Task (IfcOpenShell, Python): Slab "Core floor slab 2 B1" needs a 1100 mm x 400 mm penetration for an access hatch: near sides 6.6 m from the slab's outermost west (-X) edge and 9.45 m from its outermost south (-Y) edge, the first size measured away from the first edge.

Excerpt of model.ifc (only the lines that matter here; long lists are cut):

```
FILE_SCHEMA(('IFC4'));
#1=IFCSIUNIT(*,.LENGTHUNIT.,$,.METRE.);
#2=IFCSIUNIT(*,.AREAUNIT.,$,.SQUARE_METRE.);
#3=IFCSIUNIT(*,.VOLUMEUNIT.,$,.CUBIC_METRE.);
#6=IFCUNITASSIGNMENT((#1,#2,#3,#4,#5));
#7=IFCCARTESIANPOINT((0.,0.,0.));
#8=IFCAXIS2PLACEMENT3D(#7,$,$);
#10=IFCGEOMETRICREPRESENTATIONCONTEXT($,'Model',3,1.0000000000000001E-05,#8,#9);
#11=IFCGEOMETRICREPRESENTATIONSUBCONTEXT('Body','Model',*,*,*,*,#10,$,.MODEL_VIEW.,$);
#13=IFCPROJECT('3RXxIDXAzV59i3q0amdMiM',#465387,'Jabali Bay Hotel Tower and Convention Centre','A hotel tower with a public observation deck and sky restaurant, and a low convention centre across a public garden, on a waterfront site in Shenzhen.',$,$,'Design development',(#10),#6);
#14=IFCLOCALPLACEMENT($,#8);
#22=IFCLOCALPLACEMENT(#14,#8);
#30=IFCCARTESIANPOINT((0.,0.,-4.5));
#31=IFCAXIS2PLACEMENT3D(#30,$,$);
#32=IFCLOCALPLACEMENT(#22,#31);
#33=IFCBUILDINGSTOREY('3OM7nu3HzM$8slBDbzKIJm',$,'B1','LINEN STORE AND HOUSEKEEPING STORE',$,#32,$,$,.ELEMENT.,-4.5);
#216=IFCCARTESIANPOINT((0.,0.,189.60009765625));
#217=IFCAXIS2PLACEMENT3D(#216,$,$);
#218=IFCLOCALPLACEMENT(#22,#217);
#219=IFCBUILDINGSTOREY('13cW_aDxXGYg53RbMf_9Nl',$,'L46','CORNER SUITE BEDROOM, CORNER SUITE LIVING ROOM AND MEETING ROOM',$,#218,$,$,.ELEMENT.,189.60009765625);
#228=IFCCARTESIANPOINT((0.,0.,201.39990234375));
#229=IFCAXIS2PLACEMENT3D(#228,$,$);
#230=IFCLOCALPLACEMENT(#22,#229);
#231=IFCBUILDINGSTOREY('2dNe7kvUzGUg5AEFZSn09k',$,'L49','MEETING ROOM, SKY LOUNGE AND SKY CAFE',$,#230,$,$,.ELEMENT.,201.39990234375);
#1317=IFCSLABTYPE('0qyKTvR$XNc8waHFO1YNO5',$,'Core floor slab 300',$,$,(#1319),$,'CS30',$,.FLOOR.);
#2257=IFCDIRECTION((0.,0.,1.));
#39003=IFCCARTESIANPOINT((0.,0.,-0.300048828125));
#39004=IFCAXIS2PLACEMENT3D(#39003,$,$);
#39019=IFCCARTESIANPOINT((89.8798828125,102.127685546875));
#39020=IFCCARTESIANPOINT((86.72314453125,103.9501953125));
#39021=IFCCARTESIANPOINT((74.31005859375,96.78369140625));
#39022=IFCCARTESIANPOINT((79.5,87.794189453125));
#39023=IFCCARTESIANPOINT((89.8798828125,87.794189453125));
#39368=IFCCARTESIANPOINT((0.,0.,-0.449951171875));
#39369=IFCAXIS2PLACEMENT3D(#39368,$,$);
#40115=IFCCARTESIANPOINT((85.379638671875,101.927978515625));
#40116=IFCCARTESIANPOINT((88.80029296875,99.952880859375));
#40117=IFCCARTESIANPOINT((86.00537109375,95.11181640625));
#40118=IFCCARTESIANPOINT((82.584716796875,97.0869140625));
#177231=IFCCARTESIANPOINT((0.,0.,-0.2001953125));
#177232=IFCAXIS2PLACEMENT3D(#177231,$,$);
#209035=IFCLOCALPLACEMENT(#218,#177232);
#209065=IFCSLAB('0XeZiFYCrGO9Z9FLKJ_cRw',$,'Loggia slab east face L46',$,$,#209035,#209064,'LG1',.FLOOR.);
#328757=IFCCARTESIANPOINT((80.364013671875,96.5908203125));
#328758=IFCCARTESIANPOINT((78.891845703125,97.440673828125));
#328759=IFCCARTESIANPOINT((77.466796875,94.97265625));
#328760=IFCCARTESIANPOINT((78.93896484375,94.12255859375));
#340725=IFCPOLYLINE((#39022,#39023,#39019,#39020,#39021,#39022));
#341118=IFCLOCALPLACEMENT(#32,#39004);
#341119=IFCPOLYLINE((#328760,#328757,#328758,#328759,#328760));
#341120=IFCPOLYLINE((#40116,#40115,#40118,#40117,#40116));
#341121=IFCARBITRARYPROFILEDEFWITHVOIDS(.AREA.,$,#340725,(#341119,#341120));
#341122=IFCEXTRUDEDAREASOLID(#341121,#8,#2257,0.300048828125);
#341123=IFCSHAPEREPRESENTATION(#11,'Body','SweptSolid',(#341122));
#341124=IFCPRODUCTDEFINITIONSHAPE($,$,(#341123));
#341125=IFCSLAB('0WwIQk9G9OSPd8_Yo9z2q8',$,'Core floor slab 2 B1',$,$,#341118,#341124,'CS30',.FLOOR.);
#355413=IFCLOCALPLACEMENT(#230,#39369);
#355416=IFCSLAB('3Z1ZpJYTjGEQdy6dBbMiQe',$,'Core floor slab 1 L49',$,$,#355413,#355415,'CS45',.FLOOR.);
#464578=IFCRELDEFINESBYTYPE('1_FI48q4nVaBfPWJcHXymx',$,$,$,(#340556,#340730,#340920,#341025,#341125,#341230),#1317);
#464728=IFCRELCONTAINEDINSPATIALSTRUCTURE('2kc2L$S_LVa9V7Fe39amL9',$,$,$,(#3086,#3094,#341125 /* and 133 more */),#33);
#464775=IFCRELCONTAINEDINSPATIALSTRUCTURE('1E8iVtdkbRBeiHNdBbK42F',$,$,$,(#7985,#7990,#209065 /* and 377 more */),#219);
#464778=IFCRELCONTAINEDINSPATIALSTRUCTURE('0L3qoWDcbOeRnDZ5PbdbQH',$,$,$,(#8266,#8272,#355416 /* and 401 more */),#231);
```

```python
import numpy as np
import ifcopenshell
import ifcopenshell.api.feature
import ifcopenshell.api.geometry
import ifcopenshell.api.root
import ifcopenshell.geom
import ifcopenshell.util.placement
import ifcopenshell.util.representation
import ifcopenshell.util.shape
import ifcopenshell.util.unit

model = ifcopenshell.open("model.ifc")
unit_scale = ifcopenshell.util.unit.calculate_unit_scale(model)
settings = ifcopenshell.geom.settings()


def volume(element):
    """Net volume in cubic metres, openings subtracted."""
    shape = ifcopenshell.geom.create_shape(settings, element)
    return ifcopenshell.util.shape.get_volume(shape.geometry)


slab = model.by_id(341125)
before = volume(slab)

# Extent in the slab's own axes, in metres. The edges named are its -X and -Y sides.
slab_shape = ifcopenshell.geom.create_shape(settings, slab)
vertices = ifcopenshell.util.shape.get_vertices(slab_shape.geometry)
x_min, y_min, bottom = vertices.min(axis=0)
top = vertices[:, 2].max()

opening = ifcopenshell.api.root.create_entity(model, ifc_class="IfcOpeningElement", name="Access hatch opening", predefined_type="OPENING")
context = ifcopenshell.util.representation.get_context(model, "Model", "Body", "MODEL_VIEW")
width, depth = 1.1, 0.4
outline = [(0.0, 0.0), (width, 0.0), (width, depth), (0.0, depth), (0.0, 0.0)]
# Overshoot both faces by 50 mm so the cut is clean.
shape = ifcopenshell.api.geometry.add_slab_representation(
    model, context=context, depth=top - bottom + 0.1, polyline=outline
)
ifcopenshell.api.geometry.assign_representation(model, product=opening, representation=shape)

matrix = ifcopenshell.util.placement.get_local_placement(slab.ObjectPlacement)
matrix[:, 3] = matrix @ np.append(np.array([x_min + 6.6, y_min + 9.45, bottom - 0.05]) / unit_scale, 1.0)
ifcopenshell.api.geometry.edit_object_placement(model, product=opening, matrix=matrix, is_si=False)
ifcopenshell.api.feature.add_feature(model, feature=opening, element=slab)

after = volume(slab)

print(f"slab volume {before:.3f} -> {after:.3f} m3")

model.write("model_rev.ifc")
```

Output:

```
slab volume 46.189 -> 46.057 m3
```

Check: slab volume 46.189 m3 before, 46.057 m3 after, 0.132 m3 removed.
